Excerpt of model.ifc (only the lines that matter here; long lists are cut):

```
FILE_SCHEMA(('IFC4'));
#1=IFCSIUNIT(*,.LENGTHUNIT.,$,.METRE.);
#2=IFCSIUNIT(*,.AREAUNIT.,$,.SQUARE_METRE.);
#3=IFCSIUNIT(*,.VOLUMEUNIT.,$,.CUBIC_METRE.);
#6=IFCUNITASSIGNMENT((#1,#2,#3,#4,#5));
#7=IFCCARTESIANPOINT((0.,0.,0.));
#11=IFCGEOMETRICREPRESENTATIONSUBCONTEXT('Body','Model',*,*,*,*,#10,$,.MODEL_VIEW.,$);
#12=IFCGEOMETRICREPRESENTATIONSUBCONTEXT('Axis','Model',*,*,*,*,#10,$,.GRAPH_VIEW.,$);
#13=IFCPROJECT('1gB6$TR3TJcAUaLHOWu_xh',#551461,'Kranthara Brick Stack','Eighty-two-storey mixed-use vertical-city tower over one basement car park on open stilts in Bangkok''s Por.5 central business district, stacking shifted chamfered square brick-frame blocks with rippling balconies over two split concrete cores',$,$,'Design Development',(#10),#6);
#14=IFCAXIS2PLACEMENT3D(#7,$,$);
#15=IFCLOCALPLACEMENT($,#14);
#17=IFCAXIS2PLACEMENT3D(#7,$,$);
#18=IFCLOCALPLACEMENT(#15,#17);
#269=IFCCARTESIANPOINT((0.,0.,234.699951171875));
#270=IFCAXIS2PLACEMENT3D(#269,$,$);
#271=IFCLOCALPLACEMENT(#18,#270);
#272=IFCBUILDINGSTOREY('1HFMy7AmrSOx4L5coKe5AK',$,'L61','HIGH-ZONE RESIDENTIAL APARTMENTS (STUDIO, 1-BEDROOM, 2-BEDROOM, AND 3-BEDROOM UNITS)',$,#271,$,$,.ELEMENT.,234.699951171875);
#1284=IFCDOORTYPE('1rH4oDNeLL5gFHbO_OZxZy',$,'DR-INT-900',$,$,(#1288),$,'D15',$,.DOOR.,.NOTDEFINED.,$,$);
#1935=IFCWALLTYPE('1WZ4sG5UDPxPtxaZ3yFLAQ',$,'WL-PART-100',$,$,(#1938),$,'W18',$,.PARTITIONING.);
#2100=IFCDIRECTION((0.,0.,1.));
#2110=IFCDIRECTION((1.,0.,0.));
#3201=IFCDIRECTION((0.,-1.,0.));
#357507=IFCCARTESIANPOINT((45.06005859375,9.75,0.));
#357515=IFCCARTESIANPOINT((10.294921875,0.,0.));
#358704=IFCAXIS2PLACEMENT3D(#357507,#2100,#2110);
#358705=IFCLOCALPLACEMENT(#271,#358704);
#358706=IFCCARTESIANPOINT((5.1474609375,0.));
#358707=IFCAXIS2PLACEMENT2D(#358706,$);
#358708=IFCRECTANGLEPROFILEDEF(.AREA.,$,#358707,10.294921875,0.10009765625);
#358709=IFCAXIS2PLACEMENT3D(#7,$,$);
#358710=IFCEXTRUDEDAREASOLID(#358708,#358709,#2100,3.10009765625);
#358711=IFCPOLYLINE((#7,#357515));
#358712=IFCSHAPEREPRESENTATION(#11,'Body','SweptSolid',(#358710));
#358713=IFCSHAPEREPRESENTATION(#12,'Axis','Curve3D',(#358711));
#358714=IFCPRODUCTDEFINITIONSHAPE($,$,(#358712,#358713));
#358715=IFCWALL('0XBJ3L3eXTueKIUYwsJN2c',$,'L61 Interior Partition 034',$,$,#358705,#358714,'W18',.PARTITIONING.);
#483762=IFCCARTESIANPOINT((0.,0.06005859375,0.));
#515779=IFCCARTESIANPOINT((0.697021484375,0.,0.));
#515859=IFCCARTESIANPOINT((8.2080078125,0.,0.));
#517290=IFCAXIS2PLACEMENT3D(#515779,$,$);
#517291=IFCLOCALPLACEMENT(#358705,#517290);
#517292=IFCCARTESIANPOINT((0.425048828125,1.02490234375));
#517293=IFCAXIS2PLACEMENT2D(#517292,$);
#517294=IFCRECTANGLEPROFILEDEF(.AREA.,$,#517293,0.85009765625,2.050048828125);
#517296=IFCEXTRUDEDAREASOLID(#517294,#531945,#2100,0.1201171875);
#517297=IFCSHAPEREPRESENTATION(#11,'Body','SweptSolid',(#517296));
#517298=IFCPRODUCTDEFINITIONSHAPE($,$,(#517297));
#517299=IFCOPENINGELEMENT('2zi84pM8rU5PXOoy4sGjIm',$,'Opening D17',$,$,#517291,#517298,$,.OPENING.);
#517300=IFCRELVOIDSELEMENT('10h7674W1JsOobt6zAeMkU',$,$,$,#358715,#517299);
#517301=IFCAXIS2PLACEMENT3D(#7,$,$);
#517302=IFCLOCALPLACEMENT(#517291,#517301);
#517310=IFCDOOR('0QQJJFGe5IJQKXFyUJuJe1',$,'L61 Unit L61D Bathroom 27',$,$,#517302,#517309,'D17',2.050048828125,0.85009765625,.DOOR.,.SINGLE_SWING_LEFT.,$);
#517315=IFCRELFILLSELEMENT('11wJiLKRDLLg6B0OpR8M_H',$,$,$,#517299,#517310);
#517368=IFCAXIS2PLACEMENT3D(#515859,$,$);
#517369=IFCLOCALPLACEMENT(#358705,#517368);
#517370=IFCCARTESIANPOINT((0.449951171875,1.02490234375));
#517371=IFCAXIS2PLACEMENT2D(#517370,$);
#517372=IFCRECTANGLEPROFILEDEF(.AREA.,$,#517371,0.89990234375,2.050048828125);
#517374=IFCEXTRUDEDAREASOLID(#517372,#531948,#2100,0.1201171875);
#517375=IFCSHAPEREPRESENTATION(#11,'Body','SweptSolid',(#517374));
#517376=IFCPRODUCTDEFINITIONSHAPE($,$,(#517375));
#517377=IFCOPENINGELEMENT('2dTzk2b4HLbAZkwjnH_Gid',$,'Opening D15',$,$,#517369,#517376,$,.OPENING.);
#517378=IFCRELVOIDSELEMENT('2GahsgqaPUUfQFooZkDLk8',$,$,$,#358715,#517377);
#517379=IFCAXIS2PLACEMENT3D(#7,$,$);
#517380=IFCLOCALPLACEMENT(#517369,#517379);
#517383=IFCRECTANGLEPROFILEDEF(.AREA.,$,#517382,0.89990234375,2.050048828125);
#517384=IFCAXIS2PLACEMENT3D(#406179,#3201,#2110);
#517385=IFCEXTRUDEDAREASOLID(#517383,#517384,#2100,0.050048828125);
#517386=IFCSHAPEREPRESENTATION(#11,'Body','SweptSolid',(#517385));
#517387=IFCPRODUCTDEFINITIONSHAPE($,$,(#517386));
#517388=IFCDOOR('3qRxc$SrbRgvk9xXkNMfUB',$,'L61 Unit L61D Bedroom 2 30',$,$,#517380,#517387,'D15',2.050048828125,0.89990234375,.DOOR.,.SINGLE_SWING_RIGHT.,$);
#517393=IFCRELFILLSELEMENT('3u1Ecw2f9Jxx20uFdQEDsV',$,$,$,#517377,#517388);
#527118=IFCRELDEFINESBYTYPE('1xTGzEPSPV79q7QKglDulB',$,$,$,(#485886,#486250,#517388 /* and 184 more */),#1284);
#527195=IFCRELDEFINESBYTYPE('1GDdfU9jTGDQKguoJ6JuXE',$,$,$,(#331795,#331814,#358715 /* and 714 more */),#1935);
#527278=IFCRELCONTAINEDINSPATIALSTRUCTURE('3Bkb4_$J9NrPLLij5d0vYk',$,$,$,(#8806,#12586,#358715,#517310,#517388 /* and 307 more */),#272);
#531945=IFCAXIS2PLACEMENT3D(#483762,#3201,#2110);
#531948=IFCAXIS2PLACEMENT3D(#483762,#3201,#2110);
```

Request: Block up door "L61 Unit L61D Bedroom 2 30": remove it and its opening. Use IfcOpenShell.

```python
import ifcopenshell
import ifcopenshell.api.feature
import ifcopenshell.api.root
import ifcopenshell.geom
import ifcopenshell.util.shape

model = ifcopenshell.open("model.ifc")
settings = ifcopenshell.geom.settings()


def volume(element):
    """Net volume in cubic metres, openings subtracted."""
    shape = ifcopenshell.geom.create_shape(settings, element)
    return ifcopenshell.util.shape.get_volume(shape.geometry)


door = model.by_guid("3qRxc$SrbRgvk9xXkNMfUB")
opening = door.FillsVoids[0].RelatingOpeningElement
wall = opening.VoidsElements[0].RelatingBuildingElement
before = volume(wall)

ifcopenshell.api.root.remove_product(model, product=door)
ifcopenshell.api.feature.remove_feature(model, feature=opening)

after = volume(wall)

print(f"wall volume {before:.3f} -> {after:.3f} m3")

model.write("model_v2.ifc")
```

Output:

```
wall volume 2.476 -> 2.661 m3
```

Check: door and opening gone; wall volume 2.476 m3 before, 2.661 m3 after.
